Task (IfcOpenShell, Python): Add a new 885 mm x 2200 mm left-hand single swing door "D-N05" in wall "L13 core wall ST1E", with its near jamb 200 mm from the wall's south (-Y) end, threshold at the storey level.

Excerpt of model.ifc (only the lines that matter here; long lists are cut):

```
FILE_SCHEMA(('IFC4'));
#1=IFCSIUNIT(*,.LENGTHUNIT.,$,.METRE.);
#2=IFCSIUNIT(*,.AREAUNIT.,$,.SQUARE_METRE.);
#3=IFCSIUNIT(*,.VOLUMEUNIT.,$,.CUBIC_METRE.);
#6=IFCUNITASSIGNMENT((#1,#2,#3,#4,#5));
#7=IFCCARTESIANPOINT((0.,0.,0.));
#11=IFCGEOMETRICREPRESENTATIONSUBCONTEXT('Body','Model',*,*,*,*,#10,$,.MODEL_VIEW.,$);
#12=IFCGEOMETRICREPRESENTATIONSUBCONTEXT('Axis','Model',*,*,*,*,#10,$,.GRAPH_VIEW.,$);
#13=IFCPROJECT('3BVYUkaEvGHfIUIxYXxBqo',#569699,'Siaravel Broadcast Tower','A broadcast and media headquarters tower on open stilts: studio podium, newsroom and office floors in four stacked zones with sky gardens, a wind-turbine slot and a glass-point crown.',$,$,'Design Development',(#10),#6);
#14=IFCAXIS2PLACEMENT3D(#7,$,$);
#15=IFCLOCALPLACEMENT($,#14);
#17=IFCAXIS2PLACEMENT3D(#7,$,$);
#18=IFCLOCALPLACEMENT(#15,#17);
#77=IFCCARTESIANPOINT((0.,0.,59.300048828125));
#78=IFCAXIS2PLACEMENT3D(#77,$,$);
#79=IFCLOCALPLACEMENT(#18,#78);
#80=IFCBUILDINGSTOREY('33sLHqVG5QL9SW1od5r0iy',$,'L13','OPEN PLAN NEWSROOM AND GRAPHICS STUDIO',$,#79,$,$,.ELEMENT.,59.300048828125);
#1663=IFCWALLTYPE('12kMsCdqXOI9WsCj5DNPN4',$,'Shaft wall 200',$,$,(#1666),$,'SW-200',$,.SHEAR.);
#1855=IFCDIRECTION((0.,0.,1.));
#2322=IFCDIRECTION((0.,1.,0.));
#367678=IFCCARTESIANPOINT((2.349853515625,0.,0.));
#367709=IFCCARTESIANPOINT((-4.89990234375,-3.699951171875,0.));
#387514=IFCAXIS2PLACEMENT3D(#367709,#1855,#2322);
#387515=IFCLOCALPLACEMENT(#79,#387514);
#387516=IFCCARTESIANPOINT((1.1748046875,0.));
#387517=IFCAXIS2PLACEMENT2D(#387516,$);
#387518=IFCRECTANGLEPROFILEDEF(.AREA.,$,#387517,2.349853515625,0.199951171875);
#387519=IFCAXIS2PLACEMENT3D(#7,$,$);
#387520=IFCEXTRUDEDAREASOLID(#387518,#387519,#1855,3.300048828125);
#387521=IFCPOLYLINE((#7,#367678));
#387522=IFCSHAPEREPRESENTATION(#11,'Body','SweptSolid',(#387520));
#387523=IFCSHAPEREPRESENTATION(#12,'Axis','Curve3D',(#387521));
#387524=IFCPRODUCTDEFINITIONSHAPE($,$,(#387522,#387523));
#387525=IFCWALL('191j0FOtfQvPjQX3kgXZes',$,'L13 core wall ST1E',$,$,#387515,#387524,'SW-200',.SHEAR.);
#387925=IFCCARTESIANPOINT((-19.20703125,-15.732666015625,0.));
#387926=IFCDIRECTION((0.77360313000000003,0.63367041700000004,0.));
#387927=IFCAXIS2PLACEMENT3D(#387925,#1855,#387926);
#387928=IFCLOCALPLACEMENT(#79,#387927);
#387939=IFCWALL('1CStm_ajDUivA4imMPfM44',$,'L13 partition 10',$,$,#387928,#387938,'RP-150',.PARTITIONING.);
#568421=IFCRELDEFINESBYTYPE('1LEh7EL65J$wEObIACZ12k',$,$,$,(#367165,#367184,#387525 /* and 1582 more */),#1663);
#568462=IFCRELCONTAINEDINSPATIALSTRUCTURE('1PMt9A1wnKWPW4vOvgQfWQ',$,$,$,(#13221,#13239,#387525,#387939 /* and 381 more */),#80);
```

```python
import numpy as np
import ifcopenshell
import ifcopenshell.api.feature
import ifcopenshell.api.geometry
import ifcopenshell.api.root
import ifcopenshell.api.spatial
import ifcopenshell.geom
import ifcopenshell.util.element
import ifcopenshell.util.placement
import ifcopenshell.util.representation
import ifcopenshell.util.shape
import ifcopenshell.util.unit

model = ifcopenshell.open("model.ifc")
unit_scale = ifcopenshell.util.unit.calculate_unit_scale(model)
settings = ifcopenshell.geom.settings()


def volume(element):
    """Net volume in cubic metres, openings subtracted."""
    shape = ifcopenshell.geom.create_shape(settings, element)
    return ifcopenshell.util.shape.get_volume(shape.geometry)


wall = model.by_guid("191j0FOtfQvPjQX3kgXZes")
storey = ifcopenshell.util.element.get_container(wall, ifc_class="IfcBuildingStorey")
context = ifcopenshell.util.representation.get_context(model, "Model", "Body", "MODEL_VIEW")
before = volume(wall)

width, height, from_end, sill = 0.885, 2.2, 0.2, 0.0  # metres

# The wall runs along its own X axis, and the end named is its -X end.
wall_shape = ifcopenshell.geom.create_shape(settings, wall)
x, y, z = ifcopenshell.util.shape.get_vertices(wall_shape.geometry).T
start = x.min() + from_end
face, thickness = float(y.min()), float(y.max() - y.min())
wall_matrix = ifcopenshell.util.placement.get_local_placement(wall.ObjectPlacement)
level = ifcopenshell.util.placement.get_local_placement(storey.ObjectPlacement)[2, 3]


def in_wall(x, y):
    """Placement at x, y metres in the wall's axes, at sill height."""
    matrix = wall_matrix.copy()
    matrix[:, 3] = wall_matrix @ np.array([x / unit_scale, y / unit_scale, 0.0, 1.0])
    matrix[2, 3] = level + sill / unit_scale
    return matrix


# Opening: a box that overshoots both wall faces by 50 mm.
opening = ifcopenshell.api.root.create_entity(model, ifc_class="IfcOpeningElement", predefined_type="OPENING")
box = ifcopenshell.api.geometry.add_wall_representation(
    model, context=context, length=width, height=height, thickness=thickness + 0.1
)
ifcopenshell.api.geometry.assign_representation(model, product=opening, representation=box)
ifcopenshell.api.geometry.edit_object_placement(model, product=opening, matrix=in_wall(start, face - 0.05), is_si=False)
ifcopenshell.api.feature.add_feature(model, feature=opening, element=wall)

door = ifcopenshell.api.root.create_entity(model, ifc_class="IfcDoor", name="D-N05", predefined_type="DOOR")
door.OverallWidth, door.OverallHeight = width / unit_scale, height / unit_scale
door.OperationType = "SINGLE_SWING_LEFT"
body = ifcopenshell.api.geometry.add_door_representation(
    model,
    context=context,
    overall_width=door.OverallWidth,
    overall_height=door.OverallHeight,
    operation_type="SINGLE_SWING_LEFT",
    lining_properties={"LiningDepth": thickness / unit_scale, "ThresholdDepth": thickness / unit_scale},
)
ifcopenshell.api.geometry.assign_representation(model, product=door, representation=body)
ifcopenshell.api.spatial.assign_container(model, products=[door], relating_structure=storey)
ifcopenshell.api.feature.add_filling(model, opening=opening, element=door)

# The lining spans the wall, so the door starts at the wall face.
ifcopenshell.api.geometry.edit_object_placement(model, product=door, matrix=in_wall(start, face), is_si=False)

after = volume(wall)

print(f"wall volume {before:.3f} -> {after:.3f} m3")

model.write("model_updated.ifc")
```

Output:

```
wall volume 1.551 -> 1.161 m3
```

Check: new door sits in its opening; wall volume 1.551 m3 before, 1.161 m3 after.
